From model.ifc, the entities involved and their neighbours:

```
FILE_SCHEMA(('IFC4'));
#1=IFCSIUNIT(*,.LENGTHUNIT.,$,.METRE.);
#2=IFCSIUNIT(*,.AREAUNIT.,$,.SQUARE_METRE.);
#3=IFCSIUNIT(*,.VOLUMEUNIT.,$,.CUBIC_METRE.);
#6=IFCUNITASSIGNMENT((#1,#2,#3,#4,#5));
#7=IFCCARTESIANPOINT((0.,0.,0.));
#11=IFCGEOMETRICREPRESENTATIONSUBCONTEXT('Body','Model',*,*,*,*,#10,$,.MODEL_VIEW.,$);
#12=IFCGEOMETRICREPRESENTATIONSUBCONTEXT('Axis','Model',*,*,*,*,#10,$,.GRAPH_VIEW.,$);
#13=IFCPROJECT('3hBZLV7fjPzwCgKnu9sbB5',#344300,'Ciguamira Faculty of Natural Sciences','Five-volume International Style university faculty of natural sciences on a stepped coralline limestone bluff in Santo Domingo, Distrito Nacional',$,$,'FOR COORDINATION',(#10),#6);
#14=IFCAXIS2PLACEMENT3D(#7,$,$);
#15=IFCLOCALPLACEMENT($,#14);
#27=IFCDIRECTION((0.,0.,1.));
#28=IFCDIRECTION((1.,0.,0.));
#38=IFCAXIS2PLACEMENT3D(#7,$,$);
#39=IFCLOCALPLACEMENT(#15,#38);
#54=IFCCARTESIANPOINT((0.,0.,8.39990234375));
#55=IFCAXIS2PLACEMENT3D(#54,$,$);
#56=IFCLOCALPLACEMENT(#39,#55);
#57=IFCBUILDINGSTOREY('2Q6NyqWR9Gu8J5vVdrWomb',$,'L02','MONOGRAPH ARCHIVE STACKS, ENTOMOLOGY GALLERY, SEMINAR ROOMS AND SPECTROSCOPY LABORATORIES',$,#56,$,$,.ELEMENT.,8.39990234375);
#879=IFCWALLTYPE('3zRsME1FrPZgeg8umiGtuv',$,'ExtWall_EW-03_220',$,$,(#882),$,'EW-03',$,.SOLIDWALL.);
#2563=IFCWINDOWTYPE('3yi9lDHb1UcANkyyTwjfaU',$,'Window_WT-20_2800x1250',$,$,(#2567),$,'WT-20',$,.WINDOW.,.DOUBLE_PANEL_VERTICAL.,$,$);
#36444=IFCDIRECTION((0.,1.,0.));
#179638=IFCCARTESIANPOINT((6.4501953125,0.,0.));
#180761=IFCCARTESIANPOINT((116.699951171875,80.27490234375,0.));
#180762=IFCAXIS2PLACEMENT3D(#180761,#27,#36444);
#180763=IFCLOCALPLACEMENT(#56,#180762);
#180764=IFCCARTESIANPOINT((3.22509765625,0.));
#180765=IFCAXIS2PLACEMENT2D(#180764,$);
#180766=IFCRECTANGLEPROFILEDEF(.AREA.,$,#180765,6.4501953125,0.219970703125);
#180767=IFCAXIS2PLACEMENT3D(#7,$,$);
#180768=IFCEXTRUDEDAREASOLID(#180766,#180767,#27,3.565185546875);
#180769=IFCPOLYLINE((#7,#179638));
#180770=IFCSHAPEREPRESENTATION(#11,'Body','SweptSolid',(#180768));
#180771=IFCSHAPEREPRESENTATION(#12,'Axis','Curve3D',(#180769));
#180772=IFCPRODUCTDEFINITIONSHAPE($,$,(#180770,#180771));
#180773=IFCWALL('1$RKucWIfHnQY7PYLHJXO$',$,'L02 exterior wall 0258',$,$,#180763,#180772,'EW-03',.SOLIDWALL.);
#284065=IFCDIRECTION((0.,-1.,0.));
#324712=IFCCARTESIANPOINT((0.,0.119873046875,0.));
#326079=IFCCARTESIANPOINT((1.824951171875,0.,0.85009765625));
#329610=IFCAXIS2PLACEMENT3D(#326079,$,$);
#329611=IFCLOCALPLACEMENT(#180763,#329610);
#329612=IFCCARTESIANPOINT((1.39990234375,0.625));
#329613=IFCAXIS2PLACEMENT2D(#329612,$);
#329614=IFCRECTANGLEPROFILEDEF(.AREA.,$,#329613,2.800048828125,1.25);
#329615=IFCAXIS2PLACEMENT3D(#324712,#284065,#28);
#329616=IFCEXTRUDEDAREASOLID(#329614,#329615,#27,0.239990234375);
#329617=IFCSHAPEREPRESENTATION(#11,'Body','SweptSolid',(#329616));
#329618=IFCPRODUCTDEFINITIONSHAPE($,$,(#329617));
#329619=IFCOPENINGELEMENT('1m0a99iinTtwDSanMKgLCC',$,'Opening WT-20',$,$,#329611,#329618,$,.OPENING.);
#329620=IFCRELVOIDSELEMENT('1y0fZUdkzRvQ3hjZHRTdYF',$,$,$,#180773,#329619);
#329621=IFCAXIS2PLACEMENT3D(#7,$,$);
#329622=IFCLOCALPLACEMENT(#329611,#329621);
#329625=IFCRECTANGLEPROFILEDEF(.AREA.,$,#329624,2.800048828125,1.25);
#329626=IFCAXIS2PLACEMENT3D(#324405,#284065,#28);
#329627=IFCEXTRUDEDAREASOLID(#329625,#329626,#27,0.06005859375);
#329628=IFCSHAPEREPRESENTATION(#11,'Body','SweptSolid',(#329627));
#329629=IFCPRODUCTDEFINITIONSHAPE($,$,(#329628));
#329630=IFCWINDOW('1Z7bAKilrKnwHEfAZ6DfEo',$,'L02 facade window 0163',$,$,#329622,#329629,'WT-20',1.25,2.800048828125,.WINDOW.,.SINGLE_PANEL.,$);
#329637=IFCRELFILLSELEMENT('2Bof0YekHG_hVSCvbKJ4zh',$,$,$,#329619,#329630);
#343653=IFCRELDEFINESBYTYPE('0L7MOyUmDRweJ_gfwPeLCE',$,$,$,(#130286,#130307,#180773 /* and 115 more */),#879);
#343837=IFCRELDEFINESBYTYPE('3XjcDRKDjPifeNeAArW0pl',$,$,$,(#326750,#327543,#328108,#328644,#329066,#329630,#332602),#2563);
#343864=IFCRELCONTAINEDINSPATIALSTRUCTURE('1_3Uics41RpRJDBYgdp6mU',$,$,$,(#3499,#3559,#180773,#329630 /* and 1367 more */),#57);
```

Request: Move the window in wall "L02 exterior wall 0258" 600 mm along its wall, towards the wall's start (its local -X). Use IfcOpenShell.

```python
import ifcopenshell
import ifcopenshell.api.geometry
import ifcopenshell.util.placement

model = ifcopenshell.open("model.ifc")

window = model.by_guid("1Z7bAKilrKnwHEfAZ6DfEo")
opening = window.FillsVoids[0].RelatingOpeningElement
wall = opening.VoidsElements[0].RelatingBuildingElement

wall_matrix = ifcopenshell.util.placement.get_local_placement(wall.ObjectPlacement)
shift = wall_matrix[:3, 0] * -0.6
before = ifcopenshell.util.placement.get_local_placement(window.ObjectPlacement)[:3, 3].copy()

# The window is placed relative to its opening, so it follows when the opening moves.
matrix = ifcopenshell.util.placement.get_local_placement(opening.ObjectPlacement)
matrix[:3, 3] += shift
ifcopenshell.api.geometry.edit_object_placement(
    model, product=opening, matrix=matrix, is_si=False, should_transform_children=True
)

after = ifcopenshell.util.placement.get_local_placement(window.ObjectPlacement)[:3, 3]
print("window moved by", (after - before).round(3) + 0.0)

model.write("model_rev.ifc")
```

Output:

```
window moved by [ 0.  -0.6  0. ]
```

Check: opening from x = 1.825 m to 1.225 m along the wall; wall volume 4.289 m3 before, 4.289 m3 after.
